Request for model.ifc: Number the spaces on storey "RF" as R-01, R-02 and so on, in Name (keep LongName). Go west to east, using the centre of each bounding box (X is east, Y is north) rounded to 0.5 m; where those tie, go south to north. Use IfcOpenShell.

First a look at what the model holds.

```python
import ifcopenshell
import ifcopenshell.util.element
import ifcopenshell.util.placement

model = ifcopenshell.open("model.ifc")
print(model.schema)
storey = next(s for s in model.by_type("IfcBuildingStorey") if s.Name == "RF")
spaces = [e for e in ifcopenshell.util.element.get_decomposition(storey) if e.is_a("IfcSpace")]
for e in sorted(spaces, key=lambda e: e.id()):
    origin = ifcopenshell.util.placement.get_local_placement(e.ObjectPlacement)[:3, 3]
    print(e.id(), e.Name, e.LongName, origin.round(2) + 0.0, sep=" | ")
```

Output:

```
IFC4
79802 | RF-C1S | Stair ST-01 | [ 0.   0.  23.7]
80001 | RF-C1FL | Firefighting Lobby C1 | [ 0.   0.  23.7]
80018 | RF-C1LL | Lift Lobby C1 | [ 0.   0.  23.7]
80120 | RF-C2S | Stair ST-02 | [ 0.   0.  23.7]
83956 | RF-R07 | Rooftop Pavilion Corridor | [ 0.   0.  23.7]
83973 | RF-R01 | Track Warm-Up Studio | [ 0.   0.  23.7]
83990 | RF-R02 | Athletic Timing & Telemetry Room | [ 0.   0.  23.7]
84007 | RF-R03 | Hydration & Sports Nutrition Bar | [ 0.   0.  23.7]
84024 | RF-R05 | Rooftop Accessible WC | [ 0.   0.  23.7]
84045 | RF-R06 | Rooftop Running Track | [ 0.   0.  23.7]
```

```python
import ifcopenshell
import ifcopenshell.geom
import ifcopenshell.util.element
import ifcopenshell.util.shape

model = ifcopenshell.open("model.ifc")
settings = ifcopenshell.geom.settings()
settings.set("use-world-coords", True)


def centre(element):
    shape = ifcopenshell.geom.create_shape(settings, element)
    return ifcopenshell.util.shape.get_bbox_centroid(shape.geometry)


storey = next(s for s in model.by_type("IfcBuildingStorey") if s.Name == "RF")
spaces = [e for e in ifcopenshell.util.element.get_decomposition(storey) if e.is_a("IfcSpace")]

# Insertion points can sit at a corner or the storey origin, so sort by the geometry (in metres).
centres = {e: centre(e) for e in spaces}
spaces.sort(key=lambda e: (round(centres[e][0] / 0.5), centres[e][1]))

for i, e in enumerate(spaces, start=1):
    number = f"R-{i:02d}"
    e.Name = number
    print(e.id(), number)

model.write("model_edited.ifc")
```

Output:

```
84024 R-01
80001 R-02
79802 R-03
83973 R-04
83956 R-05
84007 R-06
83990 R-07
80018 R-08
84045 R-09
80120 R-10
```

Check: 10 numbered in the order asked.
